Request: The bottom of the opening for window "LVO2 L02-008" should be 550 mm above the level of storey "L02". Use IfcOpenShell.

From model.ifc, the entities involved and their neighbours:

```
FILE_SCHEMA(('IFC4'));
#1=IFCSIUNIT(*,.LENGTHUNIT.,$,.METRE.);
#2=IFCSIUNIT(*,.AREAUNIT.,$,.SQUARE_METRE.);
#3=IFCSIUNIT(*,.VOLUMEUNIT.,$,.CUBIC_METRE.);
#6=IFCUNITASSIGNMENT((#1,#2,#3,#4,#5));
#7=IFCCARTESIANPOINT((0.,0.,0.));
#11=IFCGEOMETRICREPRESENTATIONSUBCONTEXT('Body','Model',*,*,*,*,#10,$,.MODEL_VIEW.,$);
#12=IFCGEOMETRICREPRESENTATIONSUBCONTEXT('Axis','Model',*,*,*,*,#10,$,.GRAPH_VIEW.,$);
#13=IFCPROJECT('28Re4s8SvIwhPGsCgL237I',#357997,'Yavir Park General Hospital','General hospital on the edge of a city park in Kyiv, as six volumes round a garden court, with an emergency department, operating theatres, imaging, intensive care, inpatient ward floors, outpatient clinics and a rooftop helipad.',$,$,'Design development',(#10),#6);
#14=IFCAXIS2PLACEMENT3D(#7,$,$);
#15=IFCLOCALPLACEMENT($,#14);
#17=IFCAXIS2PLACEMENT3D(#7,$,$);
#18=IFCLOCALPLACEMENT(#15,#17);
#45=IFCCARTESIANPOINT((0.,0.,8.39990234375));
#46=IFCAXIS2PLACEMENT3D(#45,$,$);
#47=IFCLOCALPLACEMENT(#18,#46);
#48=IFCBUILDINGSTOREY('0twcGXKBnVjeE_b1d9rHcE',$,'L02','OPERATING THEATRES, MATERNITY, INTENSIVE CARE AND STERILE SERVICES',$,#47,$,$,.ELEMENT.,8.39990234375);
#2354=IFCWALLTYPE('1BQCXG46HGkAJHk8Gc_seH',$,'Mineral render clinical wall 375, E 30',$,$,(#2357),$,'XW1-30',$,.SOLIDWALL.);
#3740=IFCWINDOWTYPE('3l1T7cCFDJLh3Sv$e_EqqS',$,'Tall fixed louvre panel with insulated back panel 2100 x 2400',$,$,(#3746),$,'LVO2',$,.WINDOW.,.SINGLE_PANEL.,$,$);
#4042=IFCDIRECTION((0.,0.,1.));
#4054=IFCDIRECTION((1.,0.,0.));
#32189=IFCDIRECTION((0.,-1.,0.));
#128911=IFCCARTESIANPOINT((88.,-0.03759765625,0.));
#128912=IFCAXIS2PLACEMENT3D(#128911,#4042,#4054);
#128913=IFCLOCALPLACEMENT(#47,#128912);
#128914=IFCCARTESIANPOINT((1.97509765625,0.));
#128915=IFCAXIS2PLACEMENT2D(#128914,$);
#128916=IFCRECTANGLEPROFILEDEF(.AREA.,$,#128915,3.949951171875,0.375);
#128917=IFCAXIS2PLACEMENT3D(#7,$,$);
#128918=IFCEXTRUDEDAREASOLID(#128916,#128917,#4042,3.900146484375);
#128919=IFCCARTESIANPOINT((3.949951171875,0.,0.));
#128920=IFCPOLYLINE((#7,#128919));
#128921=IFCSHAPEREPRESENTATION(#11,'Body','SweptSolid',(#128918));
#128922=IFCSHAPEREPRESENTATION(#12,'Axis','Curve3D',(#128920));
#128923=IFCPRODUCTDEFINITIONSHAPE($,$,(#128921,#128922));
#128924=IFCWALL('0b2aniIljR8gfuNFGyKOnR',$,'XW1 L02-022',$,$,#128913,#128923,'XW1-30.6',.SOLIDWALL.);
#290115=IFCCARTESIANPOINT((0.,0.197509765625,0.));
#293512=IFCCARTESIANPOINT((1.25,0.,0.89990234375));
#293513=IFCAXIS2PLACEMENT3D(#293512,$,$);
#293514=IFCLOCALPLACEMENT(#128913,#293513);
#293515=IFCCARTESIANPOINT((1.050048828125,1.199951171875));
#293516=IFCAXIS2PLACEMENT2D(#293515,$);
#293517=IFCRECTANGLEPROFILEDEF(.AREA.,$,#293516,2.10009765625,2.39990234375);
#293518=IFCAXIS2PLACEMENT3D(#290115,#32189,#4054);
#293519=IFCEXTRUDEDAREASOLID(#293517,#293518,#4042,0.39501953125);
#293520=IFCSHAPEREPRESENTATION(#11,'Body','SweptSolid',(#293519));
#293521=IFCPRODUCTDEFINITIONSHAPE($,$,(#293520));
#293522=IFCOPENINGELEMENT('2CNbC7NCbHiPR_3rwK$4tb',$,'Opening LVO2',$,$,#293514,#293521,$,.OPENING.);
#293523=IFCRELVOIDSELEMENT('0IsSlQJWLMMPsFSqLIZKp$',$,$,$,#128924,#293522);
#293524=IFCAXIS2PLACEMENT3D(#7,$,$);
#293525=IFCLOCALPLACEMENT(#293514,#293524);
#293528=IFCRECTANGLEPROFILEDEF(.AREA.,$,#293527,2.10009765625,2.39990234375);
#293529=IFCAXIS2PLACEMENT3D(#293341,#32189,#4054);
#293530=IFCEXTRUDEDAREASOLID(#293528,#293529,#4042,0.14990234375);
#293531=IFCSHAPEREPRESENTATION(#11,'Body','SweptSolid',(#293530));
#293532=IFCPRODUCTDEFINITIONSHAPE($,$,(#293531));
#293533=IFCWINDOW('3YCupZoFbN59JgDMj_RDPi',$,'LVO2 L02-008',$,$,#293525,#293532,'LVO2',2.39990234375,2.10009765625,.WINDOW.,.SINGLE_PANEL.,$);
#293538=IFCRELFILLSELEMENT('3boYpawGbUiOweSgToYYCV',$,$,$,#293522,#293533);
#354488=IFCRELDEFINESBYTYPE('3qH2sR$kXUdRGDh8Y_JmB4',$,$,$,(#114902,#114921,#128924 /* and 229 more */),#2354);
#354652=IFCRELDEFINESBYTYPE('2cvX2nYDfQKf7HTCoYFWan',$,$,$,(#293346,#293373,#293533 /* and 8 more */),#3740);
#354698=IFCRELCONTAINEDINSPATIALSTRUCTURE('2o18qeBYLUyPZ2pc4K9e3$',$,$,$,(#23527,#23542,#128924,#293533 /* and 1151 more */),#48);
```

```python
import numpy as np
import ifcopenshell
import ifcopenshell.api.geometry
import ifcopenshell.geom
import ifcopenshell.util.element
import ifcopenshell.util.placement
import ifcopenshell.util.shape
import ifcopenshell.util.unit

model = ifcopenshell.open("model.ifc")
unit_scale = ifcopenshell.util.unit.calculate_unit_scale(model)

window = model.by_guid("3YCupZoFbN59JgDMj_RDPi")
opening = window.FillsVoids[0].RelatingOpeningElement
storey = ifcopenshell.util.element.get_container(window, ifc_class="IfcBuildingStorey")
level = ifcopenshell.util.placement.get_local_placement(storey.ObjectPlacement)[2, 3]

# The opening's origin need not be at the sill, so measure its lowest point.
shape = ifcopenshell.geom.create_shape(ifcopenshell.geom.settings(), opening)
bottom = ifcopenshell.util.shape.get_shape_bottom_elevation(shape, shape.geometry) / unit_scale
dz = level + 0.55 - bottom

shift = np.array([0.0, 0.0, dz])
# The window is placed relative to its opening, so it follows when the opening moves.
matrix = ifcopenshell.util.placement.get_local_placement(opening.ObjectPlacement)
matrix[:3, 3] += shift
ifcopenshell.api.geometry.edit_object_placement(
    model, product=opening, matrix=matrix, is_si=False, should_transform_children=True
)

print(f"moved by {dz * unit_scale:+.3f} m")

model.write("model_rev.ifc")
```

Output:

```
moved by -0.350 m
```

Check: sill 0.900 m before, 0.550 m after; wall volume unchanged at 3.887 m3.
